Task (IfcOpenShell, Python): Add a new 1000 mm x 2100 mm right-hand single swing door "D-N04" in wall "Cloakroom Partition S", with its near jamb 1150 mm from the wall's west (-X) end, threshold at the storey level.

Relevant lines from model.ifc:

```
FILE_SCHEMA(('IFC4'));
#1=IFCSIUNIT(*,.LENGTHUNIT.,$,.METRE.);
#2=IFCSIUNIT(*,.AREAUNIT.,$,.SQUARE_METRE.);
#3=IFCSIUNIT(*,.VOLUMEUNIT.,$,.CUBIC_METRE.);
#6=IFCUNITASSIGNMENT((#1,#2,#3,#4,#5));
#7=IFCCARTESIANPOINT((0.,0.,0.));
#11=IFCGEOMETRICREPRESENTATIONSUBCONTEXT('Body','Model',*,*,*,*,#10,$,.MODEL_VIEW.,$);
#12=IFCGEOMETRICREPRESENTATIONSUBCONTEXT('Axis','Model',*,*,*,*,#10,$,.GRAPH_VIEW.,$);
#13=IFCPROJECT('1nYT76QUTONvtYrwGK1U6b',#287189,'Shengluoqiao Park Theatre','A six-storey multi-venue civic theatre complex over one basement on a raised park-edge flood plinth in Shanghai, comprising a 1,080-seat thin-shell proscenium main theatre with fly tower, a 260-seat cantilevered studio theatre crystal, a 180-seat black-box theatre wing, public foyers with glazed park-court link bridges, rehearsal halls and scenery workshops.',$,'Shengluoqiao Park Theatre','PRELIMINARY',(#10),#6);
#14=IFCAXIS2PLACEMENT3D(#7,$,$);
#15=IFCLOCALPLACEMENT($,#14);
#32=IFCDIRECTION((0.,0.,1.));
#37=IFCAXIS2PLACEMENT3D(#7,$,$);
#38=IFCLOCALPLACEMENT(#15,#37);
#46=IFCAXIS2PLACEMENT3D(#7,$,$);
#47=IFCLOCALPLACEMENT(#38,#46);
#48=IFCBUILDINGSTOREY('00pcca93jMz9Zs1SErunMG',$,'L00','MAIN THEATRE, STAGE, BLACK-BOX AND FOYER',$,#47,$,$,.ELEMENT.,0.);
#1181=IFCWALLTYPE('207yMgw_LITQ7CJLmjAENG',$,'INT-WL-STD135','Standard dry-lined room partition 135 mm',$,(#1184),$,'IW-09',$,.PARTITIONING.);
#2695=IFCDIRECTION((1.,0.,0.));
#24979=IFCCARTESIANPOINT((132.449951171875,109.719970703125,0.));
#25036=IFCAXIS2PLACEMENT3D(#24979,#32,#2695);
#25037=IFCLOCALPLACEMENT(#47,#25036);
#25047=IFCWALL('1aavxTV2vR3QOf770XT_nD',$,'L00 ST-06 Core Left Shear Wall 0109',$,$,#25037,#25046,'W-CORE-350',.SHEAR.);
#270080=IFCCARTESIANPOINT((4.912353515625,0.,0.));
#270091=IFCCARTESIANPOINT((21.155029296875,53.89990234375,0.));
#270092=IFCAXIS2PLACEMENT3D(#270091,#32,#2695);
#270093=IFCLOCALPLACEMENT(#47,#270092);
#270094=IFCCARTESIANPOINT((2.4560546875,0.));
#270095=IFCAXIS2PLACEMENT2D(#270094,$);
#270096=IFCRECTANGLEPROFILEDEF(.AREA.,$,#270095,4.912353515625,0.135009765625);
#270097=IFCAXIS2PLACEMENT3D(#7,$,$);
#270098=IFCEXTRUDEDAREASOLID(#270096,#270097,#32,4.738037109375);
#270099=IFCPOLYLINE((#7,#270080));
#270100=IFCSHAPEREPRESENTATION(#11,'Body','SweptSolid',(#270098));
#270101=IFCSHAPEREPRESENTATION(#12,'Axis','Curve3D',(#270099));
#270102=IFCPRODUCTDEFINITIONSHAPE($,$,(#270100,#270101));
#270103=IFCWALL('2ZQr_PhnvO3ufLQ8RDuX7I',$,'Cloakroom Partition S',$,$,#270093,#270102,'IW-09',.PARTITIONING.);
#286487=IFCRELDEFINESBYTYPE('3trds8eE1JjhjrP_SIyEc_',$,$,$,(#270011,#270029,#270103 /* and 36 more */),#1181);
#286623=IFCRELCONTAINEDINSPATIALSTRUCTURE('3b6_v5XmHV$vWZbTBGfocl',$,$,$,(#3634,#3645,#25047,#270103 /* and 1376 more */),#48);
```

```python
import numpy as np
import ifcopenshell
import ifcopenshell.api.feature
import ifcopenshell.api.geometry
import ifcopenshell.api.root
import ifcopenshell.api.spatial
import ifcopenshell.geom
import ifcopenshell.util.element
import ifcopenshell.util.placement
import ifcopenshell.util.representation
import ifcopenshell.util.shape
import ifcopenshell.util.unit

model = ifcopenshell.open("model.ifc")
unit_scale = ifcopenshell.util.unit.calculate_unit_scale(model)
settings = ifcopenshell.geom.settings()


def volume(element):
    """Net volume in cubic metres, openings subtracted."""
    shape = ifcopenshell.geom.create_shape(settings, element)
    return ifcopenshell.util.shape.get_volume(shape.geometry)


wall = model.by_guid("2ZQr_PhnvO3ufLQ8RDuX7I")
storey = ifcopenshell.util.element.get_container(wall, ifc_class="IfcBuildingStorey")
context = ifcopenshell.util.representation.get_context(model, "Model", "Body", "MODEL_VIEW")
before = volume(wall)

width, height, from_end, sill = 1, 2.1, 1.15, 0.0  # metres

# The wall runs along its own X axis, and the end named is its -X end.
wall_shape = ifcopenshell.geom.create_shape(settings, wall)
x, y, z = ifcopenshell.util.shape.get_vertices(wall_shape.geometry).T
start = x.min() + from_end
face, thickness = float(y.min()), float(y.max() - y.min())
wall_matrix = ifcopenshell.util.placement.get_local_placement(wall.ObjectPlacement)
level = ifcopenshell.util.placement.get_local_placement(storey.ObjectPlacement)[2, 3]


def in_wall(x, y):
    """Placement at x, y metres in the wall's axes, at sill height."""
    matrix = wall_matrix.copy()
    matrix[:, 3] = wall_matrix @ np.array([x / unit_scale, y / unit_scale, 0.0, 1.0])
    matrix[2, 3] = level + sill / unit_scale
    return matrix


# Opening: a box that overshoots both wall faces by 50 mm.
opening = ifcopenshell.api.root.create_entity(model, ifc_class="IfcOpeningElement", predefined_type="OPENING")
box = ifcopenshell.api.geometry.add_wall_representation(
    model, context=context, length=width, height=height, thickness=thickness + 0.1
)
ifcopenshell.api.geometry.assign_representation(model, product=opening, representation=box)
ifcopenshell.api.geometry.edit_object_placement(model, product=opening, matrix=in_wall(start, face - 0.05), is_si=False)
ifcopenshell.api.feature.add_feature(model, feature=opening, element=wall)

door = ifcopenshell.api.root.create_entity(model, ifc_class="IfcDoor", name="D-N04", predefined_type="DOOR")
door.OverallWidth, door.OverallHeight = width / unit_scale, height / unit_scale
door.OperationType = "SINGLE_SWING_RIGHT"
body = ifcopenshell.api.geometry.add_door_representation(
    model,
    context=context,
    overall_width=door.OverallWidth,
    overall_height=door.OverallHeight,
    operation_type="SINGLE_SWING_RIGHT",
    lining_properties={"LiningDepth": thickness / unit_scale, "ThresholdDepth": thickness / unit_scale},
)
ifcopenshell.api.geometry.assign_representation(model, product=door, representation=body)
ifcopenshell.api.spatial.assign_container(model, products=[door], relating_structure=storey)
ifcopenshell.api.feature.add_filling(model, opening=opening, element=door)

# The lining spans the wall, so the door starts at the wall face.
ifcopenshell.api.geometry.edit_object_placement(model, product=door, matrix=in_wall(start, face), is_si=False)

after = volume(wall)

print(f"wall volume {before:.3f} -> {after:.3f} m3")

model.write("model_rev.ifc")
```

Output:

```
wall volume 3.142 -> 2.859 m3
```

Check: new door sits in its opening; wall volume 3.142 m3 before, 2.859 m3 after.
